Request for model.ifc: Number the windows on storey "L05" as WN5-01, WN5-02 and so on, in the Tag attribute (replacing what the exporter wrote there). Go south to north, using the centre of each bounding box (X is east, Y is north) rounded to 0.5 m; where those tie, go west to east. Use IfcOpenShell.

First a look at what the model holds.

```python
import ifcopenshell
import ifcopenshell.util.element
import ifcopenshell.util.placement

model = ifcopenshell.open("model.ifc")
print(model.schema)
storey = next(s for s in model.by_type("IfcBuildingStorey") if s.Name == "L05")
windows = [e for e in ifcopenshell.util.element.get_decomposition(storey) if e.is_a("IfcWindow")]
for e in sorted(windows, key=lambda e: e.id()):
    origin = ifcopenshell.util.placement.get_local_placement(e.ObjectPlacement)[:3, 3]
    print(e.id(), e.Tag, e.Name, origin.round(2) + 0.0, sep=" | ")
```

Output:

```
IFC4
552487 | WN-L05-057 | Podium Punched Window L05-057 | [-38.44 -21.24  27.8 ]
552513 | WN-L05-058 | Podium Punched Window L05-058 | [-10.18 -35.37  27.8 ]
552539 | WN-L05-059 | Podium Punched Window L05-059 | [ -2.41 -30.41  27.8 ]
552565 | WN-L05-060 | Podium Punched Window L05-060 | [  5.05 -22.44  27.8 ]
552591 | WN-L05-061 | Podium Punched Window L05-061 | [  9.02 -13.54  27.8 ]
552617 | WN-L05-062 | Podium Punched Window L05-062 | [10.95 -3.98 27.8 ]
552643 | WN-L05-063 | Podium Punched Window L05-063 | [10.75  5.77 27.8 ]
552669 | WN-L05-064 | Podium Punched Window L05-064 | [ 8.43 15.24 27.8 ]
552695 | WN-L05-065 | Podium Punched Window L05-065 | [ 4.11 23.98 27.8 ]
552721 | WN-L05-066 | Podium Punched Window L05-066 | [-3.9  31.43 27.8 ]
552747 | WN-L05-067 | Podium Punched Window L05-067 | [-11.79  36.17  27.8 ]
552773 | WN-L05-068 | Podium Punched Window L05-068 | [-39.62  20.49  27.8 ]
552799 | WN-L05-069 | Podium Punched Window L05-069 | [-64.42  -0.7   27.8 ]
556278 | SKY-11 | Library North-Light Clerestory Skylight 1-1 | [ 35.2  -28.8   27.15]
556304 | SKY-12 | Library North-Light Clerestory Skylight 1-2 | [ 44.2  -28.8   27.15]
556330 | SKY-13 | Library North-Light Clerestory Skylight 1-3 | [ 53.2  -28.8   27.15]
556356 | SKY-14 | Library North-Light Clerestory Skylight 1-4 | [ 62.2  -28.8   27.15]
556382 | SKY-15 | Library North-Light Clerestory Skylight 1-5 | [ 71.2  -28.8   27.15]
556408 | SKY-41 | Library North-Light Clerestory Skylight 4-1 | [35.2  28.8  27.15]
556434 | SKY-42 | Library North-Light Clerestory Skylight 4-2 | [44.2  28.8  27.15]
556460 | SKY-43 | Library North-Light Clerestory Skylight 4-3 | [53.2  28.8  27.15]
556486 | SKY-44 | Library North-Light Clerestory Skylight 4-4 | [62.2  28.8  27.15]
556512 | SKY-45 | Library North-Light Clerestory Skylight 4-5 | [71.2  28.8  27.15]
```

```python
import ifcopenshell
import ifcopenshell.geom
import ifcopenshell.util.element
import ifcopenshell.util.shape

model = ifcopenshell.open("model.ifc")
settings = ifcopenshell.geom.settings()
settings.set("use-world-coords", True)


def centre(element):
    shape = ifcopenshell.geom.create_shape(settings, element)
    return ifcopenshell.util.shape.get_bbox_centroid(shape.geometry)


storey = next(s for s in model.by_type("IfcBuildingStorey") if s.Name == "L05")
windows = [e for e in ifcopenshell.util.element.get_decomposition(storey) if e.is_a("IfcWindow")]

# Insertion points can sit at a corner or the storey origin, so sort by the geometry (in metres).
centres = {e: centre(e) for e in windows}
windows.sort(key=lambda e: (round(centres[e][1] / 0.5), centres[e][0]))

for i, e in enumerate(windows, start=1):
    number = f"WN5-{i:02d}"
    e.Tag = number
    print(e.id(), number)

model.write("model_updated.ifc")
```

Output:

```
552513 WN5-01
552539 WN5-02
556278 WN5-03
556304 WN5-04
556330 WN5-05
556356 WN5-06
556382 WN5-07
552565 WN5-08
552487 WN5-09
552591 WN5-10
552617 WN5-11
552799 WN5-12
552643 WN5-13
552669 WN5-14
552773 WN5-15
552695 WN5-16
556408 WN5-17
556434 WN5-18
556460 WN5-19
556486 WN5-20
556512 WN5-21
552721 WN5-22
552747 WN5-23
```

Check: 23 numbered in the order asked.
